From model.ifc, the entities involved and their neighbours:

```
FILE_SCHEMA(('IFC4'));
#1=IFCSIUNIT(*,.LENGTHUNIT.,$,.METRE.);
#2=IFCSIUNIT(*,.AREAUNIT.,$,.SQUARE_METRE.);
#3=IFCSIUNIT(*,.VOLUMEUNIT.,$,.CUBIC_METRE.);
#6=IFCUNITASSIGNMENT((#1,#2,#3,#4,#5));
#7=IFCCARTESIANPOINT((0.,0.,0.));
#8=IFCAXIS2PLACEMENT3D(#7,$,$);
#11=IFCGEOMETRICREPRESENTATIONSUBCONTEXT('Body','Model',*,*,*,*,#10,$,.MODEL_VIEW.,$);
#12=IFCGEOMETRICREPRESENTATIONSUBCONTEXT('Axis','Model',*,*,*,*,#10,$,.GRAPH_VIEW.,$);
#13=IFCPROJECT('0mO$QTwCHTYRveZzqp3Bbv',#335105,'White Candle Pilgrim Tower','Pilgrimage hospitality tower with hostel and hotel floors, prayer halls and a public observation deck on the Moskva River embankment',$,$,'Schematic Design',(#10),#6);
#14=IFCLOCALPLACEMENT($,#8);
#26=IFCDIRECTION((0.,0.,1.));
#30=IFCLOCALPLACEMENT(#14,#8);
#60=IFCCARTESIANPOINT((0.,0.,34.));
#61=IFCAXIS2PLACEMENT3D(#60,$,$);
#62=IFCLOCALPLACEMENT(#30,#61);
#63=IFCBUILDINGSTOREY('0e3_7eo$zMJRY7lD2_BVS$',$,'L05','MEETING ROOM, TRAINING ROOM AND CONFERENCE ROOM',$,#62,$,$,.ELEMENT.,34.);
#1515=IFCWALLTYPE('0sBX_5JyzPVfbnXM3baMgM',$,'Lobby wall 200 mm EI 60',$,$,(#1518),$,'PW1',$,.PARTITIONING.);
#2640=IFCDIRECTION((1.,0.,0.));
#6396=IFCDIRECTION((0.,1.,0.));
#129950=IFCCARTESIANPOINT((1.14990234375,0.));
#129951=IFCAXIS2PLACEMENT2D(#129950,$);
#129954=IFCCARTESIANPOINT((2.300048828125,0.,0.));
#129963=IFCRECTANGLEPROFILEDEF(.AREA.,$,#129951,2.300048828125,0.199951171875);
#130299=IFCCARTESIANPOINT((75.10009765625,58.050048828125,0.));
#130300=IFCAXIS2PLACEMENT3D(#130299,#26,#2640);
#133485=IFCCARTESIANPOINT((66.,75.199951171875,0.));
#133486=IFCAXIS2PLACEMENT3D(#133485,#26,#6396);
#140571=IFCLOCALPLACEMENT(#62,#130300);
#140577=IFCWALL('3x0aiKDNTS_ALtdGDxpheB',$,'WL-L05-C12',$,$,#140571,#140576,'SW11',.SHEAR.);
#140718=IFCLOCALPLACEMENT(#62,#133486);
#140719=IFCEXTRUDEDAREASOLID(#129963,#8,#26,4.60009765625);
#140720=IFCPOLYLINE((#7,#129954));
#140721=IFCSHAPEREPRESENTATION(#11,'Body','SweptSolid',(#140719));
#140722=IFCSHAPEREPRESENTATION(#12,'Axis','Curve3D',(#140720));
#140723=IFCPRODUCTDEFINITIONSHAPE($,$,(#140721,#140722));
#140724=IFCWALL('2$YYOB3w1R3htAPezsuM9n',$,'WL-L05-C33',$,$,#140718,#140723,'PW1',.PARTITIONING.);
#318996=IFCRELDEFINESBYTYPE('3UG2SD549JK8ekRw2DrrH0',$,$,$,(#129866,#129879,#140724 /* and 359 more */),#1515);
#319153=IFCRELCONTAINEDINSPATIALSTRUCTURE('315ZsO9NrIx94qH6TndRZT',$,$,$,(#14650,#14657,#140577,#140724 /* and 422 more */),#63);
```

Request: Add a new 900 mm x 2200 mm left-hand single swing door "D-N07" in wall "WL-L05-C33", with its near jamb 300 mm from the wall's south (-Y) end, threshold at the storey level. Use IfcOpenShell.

```python
import numpy as np
import ifcopenshell
import ifcopenshell.api.feature
import ifcopenshell.api.geometry
import ifcopenshell.api.root
import ifcopenshell.api.spatial
import ifcopenshell.geom
import ifcopenshell.util.element
import ifcopenshell.util.placement
import ifcopenshell.util.representation
import ifcopenshell.util.shape
import ifcopenshell.util.unit

model = ifcopenshell.open("model.ifc")
unit_scale = ifcopenshell.util.unit.calculate_unit_scale(model)
settings = ifcopenshell.geom.settings()


def volume(element):
    """Net volume in cubic metres, openings subtracted."""
    shape = ifcopenshell.geom.create_shape(settings, element)
    return ifcopenshell.util.shape.get_volume(shape.geometry)


wall = model.by_guid("2$YYOB3w1R3htAPezsuM9n")
storey = ifcopenshell.util.element.get_container(wall, ifc_class="IfcBuildingStorey")
context = ifcopenshell.util.representation.get_context(model, "Model", "Body", "MODEL_VIEW")
before = volume(wall)

width, height, from_end, sill = 0.9, 2.2, 0.3, 0.0  # metres

# The wall runs along its own X axis, and the end named is its -X end.
wall_shape = ifcopenshell.geom.create_shape(settings, wall)
x, y, z = ifcopenshell.util.shape.get_vertices(wall_shape.geometry).T
start = x.min() + from_end
face, thickness = float(y.min()), float(y.max() - y.min())
wall_matrix = ifcopenshell.util.placement.get_local_placement(wall.ObjectPlacement)
level = ifcopenshell.util.placement.get_local_placement(storey.ObjectPlacement)[2, 3]


def in_wall(x, y):
    """Placement at x, y metres in the wall's axes, at sill height."""
    matrix = wall_matrix.copy()
    matrix[:, 3] = wall_matrix @ np.array([x / unit_scale, y / unit_scale, 0.0, 1.0])
    matrix[2, 3] = level + sill / unit_scale
    return matrix


# Opening: a box that overshoots both wall faces by 50 mm.
opening = ifcopenshell.api.root.create_entity(model, ifc_class="IfcOpeningElement", predefined_type="OPENING")
box = ifcopenshell.api.geometry.add_wall_representation(
    model, context=context, length=width, height=height, thickness=thickness + 0.1
)
ifcopenshell.api.geometry.assign_representation(model, product=opening, representation=box)
ifcopenshell.api.geometry.edit_object_placement(model, product=opening, matrix=in_wall(start, face - 0.05), is_si=False)
ifcopenshell.api.feature.add_feature(model, feature=opening, element=wall)

door = ifcopenshell.api.root.create_entity(model, ifc_class="IfcDoor", name="D-N07", predefined_type="DOOR")
door.OverallWidth, door.OverallHeight = width / unit_scale, height / unit_scale
door.OperationType = "SINGLE_SWING_LEFT"
body = ifcopenshell.api.geometry.add_door_representation(
    model,
    context=context,
    overall_width=door.OverallWidth,
    overall_height=door.OverallHeight,
    operation_type="SINGLE_SWING_LEFT",
    lining_properties={"LiningDepth": thickness / unit_scale, "ThresholdDepth": thickness / unit_scale},
)
ifcopenshell.api.geometry.assign_representation(model, product=door, representation=body)
ifcopenshell.api.spatial.assign_container(model, products=[door], relating_structure=storey)
ifcopenshell.api.feature.add_filling(model, opening=opening, element=door)

# The lining spans the wall, so the door starts at the wall face.
ifcopenshell.api.geometry.edit_object_placement(model, product=door, matrix=in_wall(start, face), is_si=False)

after = volume(wall)

print(f"wall volume {before:.3f} -> {after:.3f} m3")

model.write("model_rev.ifc")
```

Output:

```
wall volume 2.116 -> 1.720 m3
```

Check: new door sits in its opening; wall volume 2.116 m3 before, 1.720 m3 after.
